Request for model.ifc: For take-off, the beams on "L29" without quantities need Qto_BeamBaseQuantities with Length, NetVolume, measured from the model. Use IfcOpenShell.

First a look at what the model holds.

```python
import ifcopenshell
import ifcopenshell.util.element
import ifcopenshell.util.unit

model = ifcopenshell.open("model.ifc")
print(model.schema)
for unit_type in ("LENGTHUNIT", "AREAUNIT", "VOLUMEUNIT"):
    print(unit_type, ifcopenshell.util.unit.calculate_unit_scale(model, unit_type))
storey = next(s for s in model.by_type("IfcBuildingStorey") if s.Name == "L29")
beams = [e for e in ifcopenshell.util.element.get_decomposition(storey) if e.is_a("IfcBeam")]
for e in sorted(beams, key=lambda e: e.id()):
    print(e.id(), e.is_a(), e.Name, list(ifcopenshell.util.element.get_psets(e, qtos_only=True)), sep=" | ")
```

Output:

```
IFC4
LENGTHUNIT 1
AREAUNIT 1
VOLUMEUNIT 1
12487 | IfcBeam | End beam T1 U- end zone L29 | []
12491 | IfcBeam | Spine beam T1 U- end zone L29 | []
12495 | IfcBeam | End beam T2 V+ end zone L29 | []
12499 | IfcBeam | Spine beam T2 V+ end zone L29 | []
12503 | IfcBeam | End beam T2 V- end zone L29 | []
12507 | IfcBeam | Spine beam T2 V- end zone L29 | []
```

```python
import ifcopenshell
import ifcopenshell.api.pset
import ifcopenshell.geom
import ifcopenshell.util.element
import ifcopenshell.util.shape
import ifcopenshell.util.unit

model = ifcopenshell.open("model.ifc")
unit_scale = ifcopenshell.util.unit.calculate_unit_scale(model)
volume_scale = ifcopenshell.util.unit.calculate_unit_scale(model, "VOLUMEUNIT")
settings = ifcopenshell.geom.settings()

storey = next(s for s in model.by_type("IfcBuildingStorey") if s.Name == "L29")
beams = [e for e in ifcopenshell.util.element.get_decomposition(storey) if e.is_a("IfcBeam")]

for e in sorted(beams, key=lambda e: e.id()):
    if ifcopenshell.util.element.get_psets(e, qtos_only=True, should_inherit=False):
        continue
    # Geometry comes back in metres, in the element's own axes.
    shape = ifcopenshell.geom.create_shape(settings, e)
    values = {
        "Length": ifcopenshell.util.shape.get_max_xyz(shape.geometry) / unit_scale,
        "NetVolume": ifcopenshell.util.shape.get_volume(shape.geometry) / volume_scale,
    }
    qto = ifcopenshell.api.pset.add_qto(model, product=e, name="Qto_BeamBaseQuantities")
    ifcopenshell.api.pset.edit_qto(model, qto=qto, properties=values)
    print(e.id(), {k: round(v, 3) for k, v in values.items()})

model.write("model-out.ifc")
```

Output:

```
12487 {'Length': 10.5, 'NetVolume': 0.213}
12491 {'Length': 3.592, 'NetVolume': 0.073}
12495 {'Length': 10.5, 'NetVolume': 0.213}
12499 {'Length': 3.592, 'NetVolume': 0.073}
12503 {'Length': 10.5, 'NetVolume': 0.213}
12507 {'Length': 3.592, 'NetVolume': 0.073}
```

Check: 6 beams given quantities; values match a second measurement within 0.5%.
